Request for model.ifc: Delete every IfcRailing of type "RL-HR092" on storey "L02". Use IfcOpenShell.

First a look at what the model holds.

```python
import ifcopenshell
import ifcopenshell.util.element

model = ifcopenshell.open("model.ifc")
print(model.schema)
storey = next(s for s in model.by_type("IfcBuildingStorey") if s.Name == "L02")
railings = [e for e in ifcopenshell.util.element.get_decomposition(storey) if e.is_a("IfcRailing")]
seen = {}
for e in railings:
    element_type = ifcopenshell.util.element.get_type(e)
    name = element_type.Name if element_type not in (None, e) else None
    seen[name] = seen.get(name, 0) + 1
for name, count in sorted(seen.items(), key=str):
    print(count, "x", name)
```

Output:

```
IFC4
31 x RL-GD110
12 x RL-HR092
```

```python
import ifcopenshell
import ifcopenshell.api.root
import ifcopenshell.util.element

model = ifcopenshell.open("model.ifc")

storey = next(s for s in model.by_type("IfcBuildingStorey") if s.Name == "L02")
railings = [e for e in ifcopenshell.util.element.get_decomposition(storey) if e.is_a("IfcRailing")]
targets = [e for e in railings if (t := ifcopenshell.util.element.get_type(e)) not in (None, e) and t.Name == "RL-HR092"]

for e in targets:
    ifcopenshell.api.root.remove_product(model, product=e)
print(len(targets), "removed")

model.write("model_edited.ifc")
```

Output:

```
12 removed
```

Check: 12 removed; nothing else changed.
